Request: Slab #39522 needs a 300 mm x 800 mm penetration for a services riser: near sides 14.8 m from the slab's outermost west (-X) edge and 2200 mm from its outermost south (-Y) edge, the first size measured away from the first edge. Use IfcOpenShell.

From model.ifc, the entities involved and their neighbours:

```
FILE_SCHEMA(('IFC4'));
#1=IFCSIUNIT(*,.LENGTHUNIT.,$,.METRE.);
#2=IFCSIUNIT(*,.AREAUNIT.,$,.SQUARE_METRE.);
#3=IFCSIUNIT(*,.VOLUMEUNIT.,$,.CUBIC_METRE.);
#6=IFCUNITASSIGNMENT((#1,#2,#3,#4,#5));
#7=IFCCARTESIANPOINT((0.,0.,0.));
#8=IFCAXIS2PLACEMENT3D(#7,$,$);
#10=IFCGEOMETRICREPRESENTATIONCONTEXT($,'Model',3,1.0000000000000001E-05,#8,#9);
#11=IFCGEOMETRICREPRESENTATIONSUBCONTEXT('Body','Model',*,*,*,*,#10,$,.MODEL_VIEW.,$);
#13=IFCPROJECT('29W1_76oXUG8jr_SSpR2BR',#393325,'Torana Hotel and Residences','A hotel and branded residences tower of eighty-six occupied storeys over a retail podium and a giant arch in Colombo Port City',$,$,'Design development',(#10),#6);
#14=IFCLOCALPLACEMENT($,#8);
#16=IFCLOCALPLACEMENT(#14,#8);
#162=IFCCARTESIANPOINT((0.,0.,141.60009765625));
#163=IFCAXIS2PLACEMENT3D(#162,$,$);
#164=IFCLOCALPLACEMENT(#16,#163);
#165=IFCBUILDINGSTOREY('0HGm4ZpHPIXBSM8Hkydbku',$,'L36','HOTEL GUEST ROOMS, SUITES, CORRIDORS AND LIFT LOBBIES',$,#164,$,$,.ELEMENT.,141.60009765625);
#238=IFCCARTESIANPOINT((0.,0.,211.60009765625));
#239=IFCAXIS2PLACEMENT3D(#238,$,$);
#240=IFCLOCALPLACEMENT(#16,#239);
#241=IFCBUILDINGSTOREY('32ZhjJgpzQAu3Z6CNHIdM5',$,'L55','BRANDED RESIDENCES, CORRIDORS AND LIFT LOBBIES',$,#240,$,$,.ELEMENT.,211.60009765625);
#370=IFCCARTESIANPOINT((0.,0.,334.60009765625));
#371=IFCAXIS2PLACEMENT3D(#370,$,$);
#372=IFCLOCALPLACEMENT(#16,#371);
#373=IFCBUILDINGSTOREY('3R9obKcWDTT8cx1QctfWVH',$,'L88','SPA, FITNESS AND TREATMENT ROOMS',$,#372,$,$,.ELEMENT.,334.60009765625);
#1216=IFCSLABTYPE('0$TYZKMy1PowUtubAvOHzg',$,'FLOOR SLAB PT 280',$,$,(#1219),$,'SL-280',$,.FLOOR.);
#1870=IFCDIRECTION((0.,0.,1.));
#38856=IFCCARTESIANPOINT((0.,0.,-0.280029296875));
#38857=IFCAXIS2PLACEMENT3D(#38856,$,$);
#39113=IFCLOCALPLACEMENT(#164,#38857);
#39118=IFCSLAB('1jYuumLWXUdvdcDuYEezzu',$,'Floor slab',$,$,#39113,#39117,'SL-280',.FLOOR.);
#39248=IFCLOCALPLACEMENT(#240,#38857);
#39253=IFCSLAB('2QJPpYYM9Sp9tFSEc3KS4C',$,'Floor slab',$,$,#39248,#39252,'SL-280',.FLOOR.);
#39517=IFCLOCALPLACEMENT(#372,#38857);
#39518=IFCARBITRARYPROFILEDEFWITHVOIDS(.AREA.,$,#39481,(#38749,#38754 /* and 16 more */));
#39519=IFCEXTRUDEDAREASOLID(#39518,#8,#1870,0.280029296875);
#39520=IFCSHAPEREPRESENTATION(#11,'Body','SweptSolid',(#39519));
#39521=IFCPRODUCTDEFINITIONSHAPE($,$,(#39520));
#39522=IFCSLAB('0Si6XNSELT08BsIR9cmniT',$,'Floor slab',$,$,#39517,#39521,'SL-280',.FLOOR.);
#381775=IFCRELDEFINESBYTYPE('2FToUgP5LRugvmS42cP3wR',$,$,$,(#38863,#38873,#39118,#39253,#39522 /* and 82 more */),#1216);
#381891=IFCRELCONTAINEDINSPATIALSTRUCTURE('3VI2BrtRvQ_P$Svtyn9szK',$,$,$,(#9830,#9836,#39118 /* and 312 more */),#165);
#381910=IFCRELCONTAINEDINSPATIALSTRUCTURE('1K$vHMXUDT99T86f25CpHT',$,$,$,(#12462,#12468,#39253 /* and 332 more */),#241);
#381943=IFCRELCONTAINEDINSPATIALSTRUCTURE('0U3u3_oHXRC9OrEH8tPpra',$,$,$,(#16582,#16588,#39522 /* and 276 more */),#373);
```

```python
import numpy as np
import ifcopenshell
import ifcopenshell.api.feature
import ifcopenshell.api.geometry
import ifcopenshell.api.root
import ifcopenshell.geom
import ifcopenshell.util.placement
import ifcopenshell.util.representation
import ifcopenshell.util.shape
import ifcopenshell.util.unit

model = ifcopenshell.open("model.ifc")
unit_scale = ifcopenshell.util.unit.calculate_unit_scale(model)
settings = ifcopenshell.geom.settings()


def volume(element):
    """Net volume in cubic metres, openings subtracted."""
    shape = ifcopenshell.geom.create_shape(settings, element)
    return ifcopenshell.util.shape.get_volume(shape.geometry)


slab = model.by_guid("0Si6XNSELT08BsIR9cmniT")
before = volume(slab)

# Extent in the slab's own axes, in metres. The edges named are its -X and -Y sides.
slab_shape = ifcopenshell.geom.create_shape(settings, slab)
vertices = ifcopenshell.util.shape.get_vertices(slab_shape.geometry)
x_min, y_min, bottom = vertices.min(axis=0)
top = vertices[:, 2].max()

opening = ifcopenshell.api.root.create_entity(model, ifc_class="IfcOpeningElement", name="Services riser opening", predefined_type="OPENING")
context = ifcopenshell.util.representation.get_context(model, "Model", "Body", "MODEL_VIEW")
width, depth = 0.3, 0.8
outline = [(0.0, 0.0), (width, 0.0), (width, depth), (0.0, depth), (0.0, 0.0)]
# Overshoot both faces by 50 mm so the cut is clean.
shape = ifcopenshell.api.geometry.add_slab_representation(
    model, context=context, depth=top - bottom + 0.1, polyline=outline
)
ifcopenshell.api.geometry.assign_representation(model, product=opening, representation=shape)

matrix = ifcopenshell.util.placement.get_local_placement(slab.ObjectPlacement)
matrix[:, 3] = matrix @ np.append(np.array([x_min + 14.8, y_min + 2.2, bottom - 0.05]) / unit_scale, 1.0)
ifcopenshell.api.geometry.edit_object_placement(model, product=opening, matrix=matrix, is_si=False)
ifcopenshell.api.feature.add_feature(model, feature=opening, element=slab)

after = volume(slab)

print(f"slab volume {before:.3f} -> {after:.3f} m3")

model.write("model_rev.ifc")
```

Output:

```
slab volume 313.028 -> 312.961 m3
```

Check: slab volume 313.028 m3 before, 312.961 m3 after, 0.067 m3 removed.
